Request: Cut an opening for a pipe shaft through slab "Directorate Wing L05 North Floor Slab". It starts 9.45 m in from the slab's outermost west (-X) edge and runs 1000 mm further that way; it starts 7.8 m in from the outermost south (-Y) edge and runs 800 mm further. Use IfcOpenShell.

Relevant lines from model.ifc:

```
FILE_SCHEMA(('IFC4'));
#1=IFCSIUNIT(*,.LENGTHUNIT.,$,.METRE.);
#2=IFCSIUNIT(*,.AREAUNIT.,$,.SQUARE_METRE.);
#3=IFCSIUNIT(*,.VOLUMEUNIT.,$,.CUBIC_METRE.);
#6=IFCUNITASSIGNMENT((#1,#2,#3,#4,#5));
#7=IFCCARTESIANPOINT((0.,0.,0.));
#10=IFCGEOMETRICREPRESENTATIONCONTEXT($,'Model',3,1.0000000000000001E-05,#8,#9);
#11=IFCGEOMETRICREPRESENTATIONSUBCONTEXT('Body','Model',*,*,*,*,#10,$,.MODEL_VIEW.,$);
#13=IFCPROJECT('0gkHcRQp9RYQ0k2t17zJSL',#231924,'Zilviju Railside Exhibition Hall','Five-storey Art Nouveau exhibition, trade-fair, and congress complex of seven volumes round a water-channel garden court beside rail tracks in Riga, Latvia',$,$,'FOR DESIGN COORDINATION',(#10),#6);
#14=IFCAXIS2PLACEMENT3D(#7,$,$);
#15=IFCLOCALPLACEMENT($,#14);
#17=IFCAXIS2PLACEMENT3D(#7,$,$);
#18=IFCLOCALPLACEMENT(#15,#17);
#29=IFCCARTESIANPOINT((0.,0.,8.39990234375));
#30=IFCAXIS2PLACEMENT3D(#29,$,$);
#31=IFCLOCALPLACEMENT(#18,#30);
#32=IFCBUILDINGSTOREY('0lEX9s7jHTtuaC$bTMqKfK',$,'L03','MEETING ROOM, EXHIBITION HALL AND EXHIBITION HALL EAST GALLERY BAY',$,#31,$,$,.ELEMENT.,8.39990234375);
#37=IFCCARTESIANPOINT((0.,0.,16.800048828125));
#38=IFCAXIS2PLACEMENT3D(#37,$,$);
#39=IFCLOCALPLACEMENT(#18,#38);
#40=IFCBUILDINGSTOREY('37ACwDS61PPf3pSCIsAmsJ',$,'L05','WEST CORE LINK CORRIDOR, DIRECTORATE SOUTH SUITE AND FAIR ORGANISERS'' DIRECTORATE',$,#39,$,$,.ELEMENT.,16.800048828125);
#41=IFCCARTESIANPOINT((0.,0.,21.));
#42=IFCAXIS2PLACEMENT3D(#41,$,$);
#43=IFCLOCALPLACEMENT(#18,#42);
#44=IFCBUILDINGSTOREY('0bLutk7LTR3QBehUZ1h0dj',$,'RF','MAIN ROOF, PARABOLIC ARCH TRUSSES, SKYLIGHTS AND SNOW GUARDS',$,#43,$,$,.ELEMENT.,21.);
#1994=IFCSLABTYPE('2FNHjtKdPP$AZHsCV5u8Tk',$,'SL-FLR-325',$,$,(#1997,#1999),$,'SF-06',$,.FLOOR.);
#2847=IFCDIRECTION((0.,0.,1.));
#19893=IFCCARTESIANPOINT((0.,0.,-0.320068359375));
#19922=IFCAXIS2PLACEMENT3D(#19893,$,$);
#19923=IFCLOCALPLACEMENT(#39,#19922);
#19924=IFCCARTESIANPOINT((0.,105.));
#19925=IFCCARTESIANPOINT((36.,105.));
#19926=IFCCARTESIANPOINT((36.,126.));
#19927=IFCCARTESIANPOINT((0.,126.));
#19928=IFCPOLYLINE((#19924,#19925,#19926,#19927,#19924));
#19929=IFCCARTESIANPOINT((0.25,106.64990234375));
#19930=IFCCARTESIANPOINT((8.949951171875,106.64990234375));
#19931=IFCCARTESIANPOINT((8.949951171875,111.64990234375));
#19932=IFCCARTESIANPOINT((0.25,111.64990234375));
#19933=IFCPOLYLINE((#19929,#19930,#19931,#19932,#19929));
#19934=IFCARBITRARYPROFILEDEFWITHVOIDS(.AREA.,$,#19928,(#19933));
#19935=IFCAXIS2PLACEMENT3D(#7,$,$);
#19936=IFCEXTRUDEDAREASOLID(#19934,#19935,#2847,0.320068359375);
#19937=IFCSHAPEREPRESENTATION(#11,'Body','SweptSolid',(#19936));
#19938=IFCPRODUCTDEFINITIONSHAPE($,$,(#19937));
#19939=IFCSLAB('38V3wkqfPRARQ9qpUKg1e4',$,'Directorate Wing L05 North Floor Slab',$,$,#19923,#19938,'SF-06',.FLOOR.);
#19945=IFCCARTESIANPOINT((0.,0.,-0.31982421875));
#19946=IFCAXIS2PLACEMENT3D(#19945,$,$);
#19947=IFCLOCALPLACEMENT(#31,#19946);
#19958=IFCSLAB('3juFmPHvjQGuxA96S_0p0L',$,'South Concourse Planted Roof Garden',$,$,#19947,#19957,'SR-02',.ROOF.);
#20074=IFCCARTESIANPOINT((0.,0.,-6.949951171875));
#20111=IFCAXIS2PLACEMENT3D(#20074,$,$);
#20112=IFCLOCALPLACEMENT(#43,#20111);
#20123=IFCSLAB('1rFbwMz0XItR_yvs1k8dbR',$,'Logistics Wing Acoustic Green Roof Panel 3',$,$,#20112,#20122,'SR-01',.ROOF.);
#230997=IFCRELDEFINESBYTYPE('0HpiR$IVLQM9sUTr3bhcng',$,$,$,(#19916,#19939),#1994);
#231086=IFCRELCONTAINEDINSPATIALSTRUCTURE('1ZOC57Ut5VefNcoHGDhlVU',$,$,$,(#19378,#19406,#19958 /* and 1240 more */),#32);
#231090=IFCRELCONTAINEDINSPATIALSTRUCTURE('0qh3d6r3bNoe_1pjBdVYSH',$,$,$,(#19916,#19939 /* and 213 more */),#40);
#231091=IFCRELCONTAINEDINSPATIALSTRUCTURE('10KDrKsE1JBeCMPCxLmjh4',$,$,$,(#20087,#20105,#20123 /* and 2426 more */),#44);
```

```python
import numpy as np
import ifcopenshell
import ifcopenshell.api.feature
import ifcopenshell.api.geometry
import ifcopenshell.api.root
import ifcopenshell.geom
import ifcopenshell.util.placement
import ifcopenshell.util.representation
import ifcopenshell.util.shape
import ifcopenshell.util.unit

model = ifcopenshell.open("model.ifc")
unit_scale = ifcopenshell.util.unit.calculate_unit_scale(model)
settings = ifcopenshell.geom.settings()


def volume(element):
    """Net volume in cubic metres, openings subtracted."""
    shape = ifcopenshell.geom.create_shape(settings, element)
    return ifcopenshell.util.shape.get_volume(shape.geometry)


slab = model.by_id(19939)
before = volume(slab)

# Extent in the slab's own axes, in metres. The edges named are its -X and -Y sides.
slab_shape = ifcopenshell.geom.create_shape(settings, slab)
vertices = ifcopenshell.util.shape.get_vertices(slab_shape.geometry)
x_min, y_min, bottom = vertices.min(axis=0)
top = vertices[:, 2].max()

opening = ifcopenshell.api.root.create_entity(model, ifc_class="IfcOpeningElement", name="Pipe shaft opening", predefined_type="OPENING")
context = ifcopenshell.util.representation.get_context(model, "Model", "Body", "MODEL_VIEW")
width, depth = 1, 0.8
outline = [(0.0, 0.0), (width, 0.0), (width, depth), (0.0, depth), (0.0, 0.0)]
# Overshoot both faces by 50 mm so the cut is clean.
shape = ifcopenshell.api.geometry.add_slab_representation(
    model, context=context, depth=top - bottom + 0.1, polyline=outline
)
ifcopenshell.api.geometry.assign_representation(model, product=opening, representation=shape)

matrix = ifcopenshell.util.placement.get_local_placement(slab.ObjectPlacement)
matrix[:, 3] = matrix @ np.append(np.array([x_min + 9.45, y_min + 7.8, bottom - 0.05]) / unit_scale, 1.0)
ifcopenshell.api.geometry.edit_object_placement(model, product=opening, matrix=matrix, is_si=False)
ifcopenshell.api.feature.add_feature(model, feature=opening, element=slab)

after = volume(slab)

print(f"slab volume {before:.3f} -> {after:.3f} m3")

model.write("model_edited.ifc")
```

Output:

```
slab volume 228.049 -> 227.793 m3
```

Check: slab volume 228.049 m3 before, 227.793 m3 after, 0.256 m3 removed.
